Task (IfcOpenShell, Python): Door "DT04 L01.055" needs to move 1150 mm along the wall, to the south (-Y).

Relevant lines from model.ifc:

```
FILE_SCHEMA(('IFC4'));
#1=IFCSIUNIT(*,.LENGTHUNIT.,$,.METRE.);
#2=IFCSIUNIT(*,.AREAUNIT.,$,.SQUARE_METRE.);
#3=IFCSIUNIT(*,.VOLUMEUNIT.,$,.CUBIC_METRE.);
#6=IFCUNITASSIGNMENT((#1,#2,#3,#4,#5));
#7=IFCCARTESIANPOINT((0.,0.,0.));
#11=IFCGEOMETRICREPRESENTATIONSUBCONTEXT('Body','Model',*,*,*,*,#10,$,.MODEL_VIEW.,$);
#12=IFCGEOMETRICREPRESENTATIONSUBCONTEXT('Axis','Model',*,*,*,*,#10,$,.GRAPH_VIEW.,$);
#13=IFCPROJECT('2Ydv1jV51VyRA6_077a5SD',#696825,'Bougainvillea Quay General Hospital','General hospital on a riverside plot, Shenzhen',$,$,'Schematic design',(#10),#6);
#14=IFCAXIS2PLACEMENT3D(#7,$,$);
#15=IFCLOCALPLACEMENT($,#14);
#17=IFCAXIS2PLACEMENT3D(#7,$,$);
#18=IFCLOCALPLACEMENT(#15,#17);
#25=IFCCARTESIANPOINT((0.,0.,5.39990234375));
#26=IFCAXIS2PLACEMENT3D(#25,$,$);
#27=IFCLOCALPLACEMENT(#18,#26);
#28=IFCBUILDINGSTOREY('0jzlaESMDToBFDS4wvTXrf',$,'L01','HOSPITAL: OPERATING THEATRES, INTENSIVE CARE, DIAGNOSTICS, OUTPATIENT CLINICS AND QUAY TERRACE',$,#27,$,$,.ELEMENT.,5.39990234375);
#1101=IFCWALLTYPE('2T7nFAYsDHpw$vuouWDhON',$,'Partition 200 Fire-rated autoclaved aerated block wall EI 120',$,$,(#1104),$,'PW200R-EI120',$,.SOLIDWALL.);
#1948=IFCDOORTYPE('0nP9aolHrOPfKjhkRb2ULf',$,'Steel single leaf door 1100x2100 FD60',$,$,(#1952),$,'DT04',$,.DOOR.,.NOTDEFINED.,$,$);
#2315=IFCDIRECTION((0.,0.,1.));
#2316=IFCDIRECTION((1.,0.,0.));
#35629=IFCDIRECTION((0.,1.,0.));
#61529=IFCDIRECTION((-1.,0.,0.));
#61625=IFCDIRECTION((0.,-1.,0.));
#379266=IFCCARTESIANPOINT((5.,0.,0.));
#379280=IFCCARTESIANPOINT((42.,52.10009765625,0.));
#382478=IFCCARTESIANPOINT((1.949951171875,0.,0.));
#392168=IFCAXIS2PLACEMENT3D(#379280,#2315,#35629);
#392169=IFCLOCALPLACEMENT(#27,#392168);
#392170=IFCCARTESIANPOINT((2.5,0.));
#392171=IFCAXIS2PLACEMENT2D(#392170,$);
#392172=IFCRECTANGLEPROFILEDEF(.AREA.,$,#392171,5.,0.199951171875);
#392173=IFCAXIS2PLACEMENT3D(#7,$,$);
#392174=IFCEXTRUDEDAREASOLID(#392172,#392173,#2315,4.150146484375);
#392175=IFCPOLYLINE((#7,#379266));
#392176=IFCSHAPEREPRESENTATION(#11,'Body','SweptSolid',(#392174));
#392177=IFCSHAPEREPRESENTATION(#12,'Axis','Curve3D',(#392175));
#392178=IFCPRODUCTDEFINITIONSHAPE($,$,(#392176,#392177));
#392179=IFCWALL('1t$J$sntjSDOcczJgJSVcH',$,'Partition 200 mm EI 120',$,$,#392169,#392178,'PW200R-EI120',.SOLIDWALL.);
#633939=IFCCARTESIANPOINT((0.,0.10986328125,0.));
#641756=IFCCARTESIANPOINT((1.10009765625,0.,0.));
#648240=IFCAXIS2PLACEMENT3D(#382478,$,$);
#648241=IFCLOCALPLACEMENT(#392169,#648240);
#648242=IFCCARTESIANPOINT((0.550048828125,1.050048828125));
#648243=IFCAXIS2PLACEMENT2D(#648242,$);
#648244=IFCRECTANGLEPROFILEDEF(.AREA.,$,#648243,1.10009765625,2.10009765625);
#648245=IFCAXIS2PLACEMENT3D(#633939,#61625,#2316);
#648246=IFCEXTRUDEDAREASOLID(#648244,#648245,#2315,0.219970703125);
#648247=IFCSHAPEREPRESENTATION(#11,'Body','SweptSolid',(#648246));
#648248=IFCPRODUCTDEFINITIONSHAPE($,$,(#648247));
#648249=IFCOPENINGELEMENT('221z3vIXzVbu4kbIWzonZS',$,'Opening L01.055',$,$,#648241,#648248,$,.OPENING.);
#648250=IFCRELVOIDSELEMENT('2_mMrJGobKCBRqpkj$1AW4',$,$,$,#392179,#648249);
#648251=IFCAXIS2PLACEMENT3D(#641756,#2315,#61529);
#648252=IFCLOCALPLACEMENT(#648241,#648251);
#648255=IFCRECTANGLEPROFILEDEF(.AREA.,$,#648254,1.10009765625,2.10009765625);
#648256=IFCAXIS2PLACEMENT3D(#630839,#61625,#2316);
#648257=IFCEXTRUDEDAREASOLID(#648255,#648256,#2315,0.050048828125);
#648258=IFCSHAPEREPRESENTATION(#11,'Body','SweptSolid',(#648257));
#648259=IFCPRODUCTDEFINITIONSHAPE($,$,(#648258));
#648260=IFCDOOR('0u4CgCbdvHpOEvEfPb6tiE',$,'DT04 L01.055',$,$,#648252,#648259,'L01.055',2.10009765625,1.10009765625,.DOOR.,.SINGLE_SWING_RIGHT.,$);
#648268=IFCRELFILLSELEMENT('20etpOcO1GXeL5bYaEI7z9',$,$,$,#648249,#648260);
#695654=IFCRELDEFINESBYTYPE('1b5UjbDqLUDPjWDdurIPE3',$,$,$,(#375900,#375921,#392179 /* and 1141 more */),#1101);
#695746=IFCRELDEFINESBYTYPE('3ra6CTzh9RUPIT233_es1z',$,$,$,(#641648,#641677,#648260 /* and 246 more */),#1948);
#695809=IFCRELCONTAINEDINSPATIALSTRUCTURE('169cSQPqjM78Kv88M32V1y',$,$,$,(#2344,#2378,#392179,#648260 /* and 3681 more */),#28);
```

```python
import ifcopenshell
import ifcopenshell.api.geometry
import ifcopenshell.util.placement
import ifcopenshell.util.unit

model = ifcopenshell.open("model.ifc")
unit_scale = ifcopenshell.util.unit.calculate_unit_scale(model)

door = model.by_guid("0u4CgCbdvHpOEvEfPb6tiE")
opening = door.FillsVoids[0].RelatingOpeningElement
wall = opening.VoidsElements[0].RelatingBuildingElement

wall_matrix = ifcopenshell.util.placement.get_local_placement(wall.ObjectPlacement)
shift = wall_matrix[:3, 0] * -1.15 / unit_scale
before = ifcopenshell.util.placement.get_local_placement(door.ObjectPlacement)[:3, 3].copy()

# The door is placed relative to its opening, so it follows when the opening moves.
matrix = ifcopenshell.util.placement.get_local_placement(opening.ObjectPlacement)
matrix[:3, 3] += shift
ifcopenshell.api.geometry.edit_object_placement(
    model, product=opening, matrix=matrix, is_si=False, should_transform_children=True
)

after = ifcopenshell.util.placement.get_local_placement(door.ObjectPlacement)[:3, 3]
print("door moved by", (after - before).round(3) + 0.0)

model.write("model-out.ifc")
```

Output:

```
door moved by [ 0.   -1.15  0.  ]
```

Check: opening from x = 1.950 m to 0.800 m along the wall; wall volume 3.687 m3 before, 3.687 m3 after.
